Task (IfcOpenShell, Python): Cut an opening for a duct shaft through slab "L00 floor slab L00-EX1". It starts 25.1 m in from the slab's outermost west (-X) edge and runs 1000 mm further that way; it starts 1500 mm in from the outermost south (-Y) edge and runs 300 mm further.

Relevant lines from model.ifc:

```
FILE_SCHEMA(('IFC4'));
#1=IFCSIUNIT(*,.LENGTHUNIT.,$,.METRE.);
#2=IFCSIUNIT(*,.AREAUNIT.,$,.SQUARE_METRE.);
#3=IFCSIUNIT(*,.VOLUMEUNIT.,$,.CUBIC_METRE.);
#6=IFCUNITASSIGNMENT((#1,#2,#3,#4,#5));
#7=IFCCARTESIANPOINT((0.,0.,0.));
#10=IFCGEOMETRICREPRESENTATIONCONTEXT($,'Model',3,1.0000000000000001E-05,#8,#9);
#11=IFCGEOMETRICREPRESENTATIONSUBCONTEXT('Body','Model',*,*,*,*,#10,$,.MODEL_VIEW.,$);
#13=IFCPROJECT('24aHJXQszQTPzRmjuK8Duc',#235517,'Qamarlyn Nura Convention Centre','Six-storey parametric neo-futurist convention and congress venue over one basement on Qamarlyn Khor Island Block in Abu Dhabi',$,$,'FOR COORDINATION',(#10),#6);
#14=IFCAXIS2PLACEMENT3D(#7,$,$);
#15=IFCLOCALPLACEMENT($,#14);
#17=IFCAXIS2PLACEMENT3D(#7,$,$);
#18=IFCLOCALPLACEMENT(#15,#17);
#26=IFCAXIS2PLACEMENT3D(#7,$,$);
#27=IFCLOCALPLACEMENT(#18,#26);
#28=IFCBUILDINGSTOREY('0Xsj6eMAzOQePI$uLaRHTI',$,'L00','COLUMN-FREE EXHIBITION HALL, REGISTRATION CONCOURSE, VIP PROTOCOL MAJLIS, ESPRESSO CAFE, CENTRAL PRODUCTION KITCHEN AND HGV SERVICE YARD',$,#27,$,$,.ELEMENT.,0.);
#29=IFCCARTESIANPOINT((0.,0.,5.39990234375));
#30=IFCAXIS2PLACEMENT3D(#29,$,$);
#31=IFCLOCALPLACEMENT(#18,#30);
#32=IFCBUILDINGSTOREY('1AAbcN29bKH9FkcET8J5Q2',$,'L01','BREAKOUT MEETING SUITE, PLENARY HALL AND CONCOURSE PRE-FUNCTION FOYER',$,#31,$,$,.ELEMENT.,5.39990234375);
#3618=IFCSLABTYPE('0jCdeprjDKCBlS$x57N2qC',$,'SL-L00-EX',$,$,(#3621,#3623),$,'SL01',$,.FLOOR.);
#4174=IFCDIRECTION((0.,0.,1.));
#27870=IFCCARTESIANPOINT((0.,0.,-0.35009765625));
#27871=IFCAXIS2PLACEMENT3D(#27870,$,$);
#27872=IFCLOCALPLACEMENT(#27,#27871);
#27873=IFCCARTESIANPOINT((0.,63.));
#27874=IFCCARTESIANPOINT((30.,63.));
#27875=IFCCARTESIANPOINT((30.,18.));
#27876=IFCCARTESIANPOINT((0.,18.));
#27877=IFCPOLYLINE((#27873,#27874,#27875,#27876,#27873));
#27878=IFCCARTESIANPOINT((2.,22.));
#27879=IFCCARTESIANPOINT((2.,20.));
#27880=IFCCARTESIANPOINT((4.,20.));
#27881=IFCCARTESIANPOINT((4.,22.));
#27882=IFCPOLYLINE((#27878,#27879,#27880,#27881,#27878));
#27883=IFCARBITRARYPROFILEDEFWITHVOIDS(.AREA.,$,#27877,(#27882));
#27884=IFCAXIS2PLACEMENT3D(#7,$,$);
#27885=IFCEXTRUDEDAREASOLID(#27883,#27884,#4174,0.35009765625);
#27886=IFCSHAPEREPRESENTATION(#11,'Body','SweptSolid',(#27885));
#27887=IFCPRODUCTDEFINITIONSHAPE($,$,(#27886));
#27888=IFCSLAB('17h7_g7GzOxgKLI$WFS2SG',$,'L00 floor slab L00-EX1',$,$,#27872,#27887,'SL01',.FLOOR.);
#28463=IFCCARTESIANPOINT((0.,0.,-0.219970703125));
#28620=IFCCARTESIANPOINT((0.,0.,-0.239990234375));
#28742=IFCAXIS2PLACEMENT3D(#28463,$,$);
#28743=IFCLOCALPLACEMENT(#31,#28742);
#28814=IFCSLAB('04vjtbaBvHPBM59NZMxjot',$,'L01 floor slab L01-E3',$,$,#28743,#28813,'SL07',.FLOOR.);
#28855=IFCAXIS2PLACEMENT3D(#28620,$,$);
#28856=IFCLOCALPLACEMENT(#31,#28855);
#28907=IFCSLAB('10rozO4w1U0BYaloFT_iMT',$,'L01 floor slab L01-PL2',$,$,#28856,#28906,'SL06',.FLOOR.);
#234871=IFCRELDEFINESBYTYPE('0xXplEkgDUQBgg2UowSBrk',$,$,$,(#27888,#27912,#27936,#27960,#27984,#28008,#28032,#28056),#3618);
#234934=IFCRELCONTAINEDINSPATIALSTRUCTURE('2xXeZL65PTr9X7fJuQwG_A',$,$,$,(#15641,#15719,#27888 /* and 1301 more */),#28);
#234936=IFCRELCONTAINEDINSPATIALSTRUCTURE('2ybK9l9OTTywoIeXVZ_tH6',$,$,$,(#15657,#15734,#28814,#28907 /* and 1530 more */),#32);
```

```python
import numpy as np
import ifcopenshell
import ifcopenshell.api.feature
import ifcopenshell.api.geometry
import ifcopenshell.api.root
import ifcopenshell.geom
import ifcopenshell.util.placement
import ifcopenshell.util.representation
import ifcopenshell.util.shape
import ifcopenshell.util.unit

model = ifcopenshell.open("model.ifc")
unit_scale = ifcopenshell.util.unit.calculate_unit_scale(model)
settings = ifcopenshell.geom.settings()


def volume(element):
    """Net volume in cubic metres, openings subtracted."""
    shape = ifcopenshell.geom.create_shape(settings, element)
    return ifcopenshell.util.shape.get_volume(shape.geometry)


slab = model.by_guid("17h7_g7GzOxgKLI$WFS2SG")
before = volume(slab)

# Extent in the slab's own axes, in metres. The edges named are its -X and -Y sides.
slab_shape = ifcopenshell.geom.create_shape(settings, slab)
vertices = ifcopenshell.util.shape.get_vertices(slab_shape.geometry)
x_min, y_min, bottom = vertices.min(axis=0)
top = vertices[:, 2].max()

opening = ifcopenshell.api.root.create_entity(model, ifc_class="IfcOpeningElement", name="Duct shaft opening", predefined_type="OPENING")
context = ifcopenshell.util.representation.get_context(model, "Model", "Body", "MODEL_VIEW")
width, depth = 1, 0.3
outline = [(0.0, 0.0), (width, 0.0), (width, depth), (0.0, depth), (0.0, 0.0)]
# Overshoot both faces by 50 mm so the cut is clean.
shape = ifcopenshell.api.geometry.add_slab_representation(
    model, context=context, depth=top - bottom + 0.1, polyline=outline
)
ifcopenshell.api.geometry.assign_representation(model, product=opening, representation=shape)

matrix = ifcopenshell.util.placement.get_local_placement(slab.ObjectPlacement)
matrix[:, 3] = matrix @ np.append(np.array([x_min + 25.1, y_min + 1.5, bottom - 0.05]) / unit_scale, 1.0)
ifcopenshell.api.geometry.edit_object_placement(model, product=opening, matrix=matrix, is_si=False)
ifcopenshell.api.feature.add_feature(model, feature=opening, element=slab)

after = volume(slab)

print(f"slab volume {before:.3f} -> {after:.3f} m3")

model.write("model_updated.ifc")
```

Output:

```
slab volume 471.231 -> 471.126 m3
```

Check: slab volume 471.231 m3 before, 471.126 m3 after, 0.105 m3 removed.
